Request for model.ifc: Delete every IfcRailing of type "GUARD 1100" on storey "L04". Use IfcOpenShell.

First a look at what the model holds.

```python
import ifcopenshell
import ifcopenshell.util.element

model = ifcopenshell.open("model.ifc")
print(model.schema)
storey = next(s for s in model.by_type("IfcBuildingStorey") if s.Name == "L04")
railings = [e for e in ifcopenshell.util.element.get_decomposition(storey) if e.is_a("IfcRailing")]
seen = {}
for e in railings:
    element_type = ifcopenshell.util.element.get_type(e)
    name = element_type.Name if element_type not in (None, e) else None
    seen[name] = seen.get(name, 0) + 1
for name, count in sorted(seen.items(), key=str):
    print(count, "x", name)
```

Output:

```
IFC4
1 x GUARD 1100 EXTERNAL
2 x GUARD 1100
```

```python
import ifcopenshell
import ifcopenshell.api.root
import ifcopenshell.util.element

model = ifcopenshell.open("model.ifc")

storey = next(s for s in model.by_type("IfcBuildingStorey") if s.Name == "L04")
railings = [e for e in ifcopenshell.util.element.get_decomposition(storey) if e.is_a("IfcRailing")]
targets = [e for e in railings if (t := ifcopenshell.util.element.get_type(e)) not in (None, e) and t.Name == "GUARD 1100"]

for e in targets:
    ifcopenshell.api.root.remove_product(model, product=e)
print(len(targets), "removed")

model.write("model_edited.ifc")
```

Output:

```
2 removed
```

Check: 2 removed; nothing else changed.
